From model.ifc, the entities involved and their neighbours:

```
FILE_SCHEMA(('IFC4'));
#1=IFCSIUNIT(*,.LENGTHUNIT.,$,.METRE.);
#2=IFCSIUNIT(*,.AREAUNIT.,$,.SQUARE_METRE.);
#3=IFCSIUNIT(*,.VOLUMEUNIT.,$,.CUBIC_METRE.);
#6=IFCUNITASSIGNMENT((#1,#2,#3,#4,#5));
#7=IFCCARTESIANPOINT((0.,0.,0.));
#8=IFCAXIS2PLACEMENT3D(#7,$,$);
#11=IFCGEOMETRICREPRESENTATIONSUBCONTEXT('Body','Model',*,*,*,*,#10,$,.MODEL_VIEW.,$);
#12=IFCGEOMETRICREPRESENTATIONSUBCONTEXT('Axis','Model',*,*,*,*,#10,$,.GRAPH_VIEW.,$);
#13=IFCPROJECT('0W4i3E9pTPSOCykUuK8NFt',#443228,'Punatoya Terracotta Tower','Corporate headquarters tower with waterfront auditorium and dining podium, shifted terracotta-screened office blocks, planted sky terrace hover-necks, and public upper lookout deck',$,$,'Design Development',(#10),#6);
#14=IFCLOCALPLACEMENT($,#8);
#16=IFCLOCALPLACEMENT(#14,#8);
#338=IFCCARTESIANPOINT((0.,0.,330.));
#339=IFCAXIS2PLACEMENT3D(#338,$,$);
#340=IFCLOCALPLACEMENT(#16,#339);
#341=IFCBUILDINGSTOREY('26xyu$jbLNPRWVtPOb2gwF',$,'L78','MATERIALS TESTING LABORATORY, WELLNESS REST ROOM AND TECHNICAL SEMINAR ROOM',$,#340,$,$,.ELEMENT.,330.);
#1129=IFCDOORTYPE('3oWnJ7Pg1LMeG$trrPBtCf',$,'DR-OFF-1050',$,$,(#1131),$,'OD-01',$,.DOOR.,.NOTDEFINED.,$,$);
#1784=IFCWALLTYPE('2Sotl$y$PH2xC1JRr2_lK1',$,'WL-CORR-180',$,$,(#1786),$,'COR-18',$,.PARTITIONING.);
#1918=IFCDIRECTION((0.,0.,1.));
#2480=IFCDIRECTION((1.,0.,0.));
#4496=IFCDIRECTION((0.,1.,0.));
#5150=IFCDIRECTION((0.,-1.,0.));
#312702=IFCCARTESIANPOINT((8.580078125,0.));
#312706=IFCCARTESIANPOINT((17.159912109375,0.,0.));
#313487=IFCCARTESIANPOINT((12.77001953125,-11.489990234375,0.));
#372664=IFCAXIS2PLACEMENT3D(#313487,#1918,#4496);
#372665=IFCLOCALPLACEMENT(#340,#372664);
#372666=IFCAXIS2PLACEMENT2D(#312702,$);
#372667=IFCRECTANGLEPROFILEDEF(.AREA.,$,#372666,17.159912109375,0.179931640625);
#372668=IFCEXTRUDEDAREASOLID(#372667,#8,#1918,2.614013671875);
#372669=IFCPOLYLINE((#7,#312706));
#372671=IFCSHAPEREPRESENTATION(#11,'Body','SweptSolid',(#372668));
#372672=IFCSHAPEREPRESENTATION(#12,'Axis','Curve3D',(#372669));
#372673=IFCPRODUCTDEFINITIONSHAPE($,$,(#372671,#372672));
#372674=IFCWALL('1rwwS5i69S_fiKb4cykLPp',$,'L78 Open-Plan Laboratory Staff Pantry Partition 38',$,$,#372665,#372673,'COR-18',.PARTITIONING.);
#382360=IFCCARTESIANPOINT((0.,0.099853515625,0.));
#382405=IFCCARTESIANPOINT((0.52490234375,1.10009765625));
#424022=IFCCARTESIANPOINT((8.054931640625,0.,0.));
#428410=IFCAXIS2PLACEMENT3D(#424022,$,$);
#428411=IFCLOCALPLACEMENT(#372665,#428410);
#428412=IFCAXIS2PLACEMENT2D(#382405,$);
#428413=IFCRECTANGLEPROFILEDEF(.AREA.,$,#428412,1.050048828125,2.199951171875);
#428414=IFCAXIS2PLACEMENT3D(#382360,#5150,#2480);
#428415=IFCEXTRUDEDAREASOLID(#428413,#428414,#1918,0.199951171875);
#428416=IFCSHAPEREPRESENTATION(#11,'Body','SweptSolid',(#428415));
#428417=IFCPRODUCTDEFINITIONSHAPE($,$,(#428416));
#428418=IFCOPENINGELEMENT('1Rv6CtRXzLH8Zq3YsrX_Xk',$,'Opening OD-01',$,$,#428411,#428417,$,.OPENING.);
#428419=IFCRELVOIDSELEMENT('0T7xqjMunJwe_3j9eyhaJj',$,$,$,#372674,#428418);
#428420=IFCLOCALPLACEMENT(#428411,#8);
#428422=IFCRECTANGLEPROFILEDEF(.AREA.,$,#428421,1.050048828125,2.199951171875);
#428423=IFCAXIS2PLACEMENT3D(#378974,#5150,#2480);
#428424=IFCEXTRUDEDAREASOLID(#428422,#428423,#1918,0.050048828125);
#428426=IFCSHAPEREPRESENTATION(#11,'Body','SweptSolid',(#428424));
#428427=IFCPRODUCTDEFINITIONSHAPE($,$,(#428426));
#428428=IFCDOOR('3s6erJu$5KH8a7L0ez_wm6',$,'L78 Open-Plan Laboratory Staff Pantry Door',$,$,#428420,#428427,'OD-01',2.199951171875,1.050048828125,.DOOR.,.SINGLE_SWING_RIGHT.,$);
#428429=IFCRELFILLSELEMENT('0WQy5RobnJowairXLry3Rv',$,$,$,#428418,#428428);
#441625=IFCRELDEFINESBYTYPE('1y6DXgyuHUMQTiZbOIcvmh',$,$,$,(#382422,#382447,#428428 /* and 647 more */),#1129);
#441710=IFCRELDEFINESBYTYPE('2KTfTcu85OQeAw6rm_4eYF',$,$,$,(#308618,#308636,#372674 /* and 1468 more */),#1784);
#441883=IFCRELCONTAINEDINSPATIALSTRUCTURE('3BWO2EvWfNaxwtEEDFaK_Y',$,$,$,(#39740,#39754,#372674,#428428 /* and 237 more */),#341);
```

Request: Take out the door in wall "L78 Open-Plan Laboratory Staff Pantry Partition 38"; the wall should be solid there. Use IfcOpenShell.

```python
import ifcopenshell
import ifcopenshell.api.feature
import ifcopenshell.api.root
import ifcopenshell.geom
import ifcopenshell.util.shape

model = ifcopenshell.open("model.ifc")
settings = ifcopenshell.geom.settings()


def volume(element):
    """Net volume in cubic metres, openings subtracted."""
    shape = ifcopenshell.geom.create_shape(settings, element)
    return ifcopenshell.util.shape.get_volume(shape.geometry)


door = model.by_id(428428)
opening = door.FillsVoids[0].RelatingOpeningElement
wall = opening.VoidsElements[0].RelatingBuildingElement
before = volume(wall)

ifcopenshell.api.root.remove_product(model, product=door)
ifcopenshell.api.feature.remove_feature(model, feature=opening)

after = volume(wall)

print(f"wall volume {before:.3f} -> {after:.3f} m3")

model.write("model_v2.ifc")
```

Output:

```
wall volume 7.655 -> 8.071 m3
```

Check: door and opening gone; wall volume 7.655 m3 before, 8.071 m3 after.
